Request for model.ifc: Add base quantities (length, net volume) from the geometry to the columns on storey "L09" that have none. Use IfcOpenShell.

First a look at what the model holds.

```python
import ifcopenshell
import ifcopenshell.util.element
import ifcopenshell.util.unit

model = ifcopenshell.open("model.ifc")
print(model.schema)
for unit_type in ("LENGTHUNIT", "AREAUNIT", "VOLUMEUNIT"):
    print(unit_type, ifcopenshell.util.unit.calculate_unit_scale(model, unit_type))
storey = next(s for s in model.by_type("IfcBuildingStorey") if s.Name == "L09")
columns = [e for e in ifcopenshell.util.element.get_decomposition(storey) if e.is_a("IfcColumn")]
for e in sorted(columns, key=lambda e: e.id()):
    print(e.id(), e.is_a(), e.Name, list(ifcopenshell.util.element.get_psets(e, qtos_only=True)), sep=" | ")
```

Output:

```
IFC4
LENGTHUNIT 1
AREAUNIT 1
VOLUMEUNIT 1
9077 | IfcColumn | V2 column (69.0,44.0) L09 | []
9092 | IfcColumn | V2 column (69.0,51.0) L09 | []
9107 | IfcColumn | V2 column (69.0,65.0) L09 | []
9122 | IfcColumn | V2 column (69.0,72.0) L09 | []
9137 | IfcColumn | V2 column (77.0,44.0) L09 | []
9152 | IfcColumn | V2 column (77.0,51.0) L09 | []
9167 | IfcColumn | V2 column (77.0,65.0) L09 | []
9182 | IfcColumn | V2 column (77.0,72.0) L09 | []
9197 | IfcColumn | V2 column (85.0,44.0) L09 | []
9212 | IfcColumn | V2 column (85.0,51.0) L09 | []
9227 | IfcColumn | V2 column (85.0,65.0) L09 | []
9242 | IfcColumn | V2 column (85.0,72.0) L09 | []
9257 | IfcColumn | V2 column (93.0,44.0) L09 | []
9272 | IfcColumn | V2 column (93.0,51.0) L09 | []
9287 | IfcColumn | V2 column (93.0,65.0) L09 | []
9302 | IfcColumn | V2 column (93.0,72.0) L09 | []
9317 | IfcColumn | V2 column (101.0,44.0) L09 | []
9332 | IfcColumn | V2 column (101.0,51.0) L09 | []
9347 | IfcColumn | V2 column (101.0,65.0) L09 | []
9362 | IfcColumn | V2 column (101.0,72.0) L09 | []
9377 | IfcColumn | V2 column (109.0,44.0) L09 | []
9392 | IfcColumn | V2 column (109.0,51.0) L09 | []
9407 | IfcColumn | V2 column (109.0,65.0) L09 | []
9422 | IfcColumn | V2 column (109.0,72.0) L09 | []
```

```python
import ifcopenshell
import ifcopenshell.api.pset
import ifcopenshell.geom
import ifcopenshell.util.element
import ifcopenshell.util.shape
import ifcopenshell.util.unit

model = ifcopenshell.open("model.ifc")
unit_scale = ifcopenshell.util.unit.calculate_unit_scale(model)
volume_scale = ifcopenshell.util.unit.calculate_unit_scale(model, "VOLUMEUNIT")
settings = ifcopenshell.geom.settings()

storey = next(s for s in model.by_type("IfcBuildingStorey") if s.Name == "L09")
columns = [e for e in ifcopenshell.util.element.get_decomposition(storey) if e.is_a("IfcColumn")]

for e in sorted(columns, key=lambda e: e.id()):
    if ifcopenshell.util.element.get_psets(e, qtos_only=True, should_inherit=False):
        continue
    # Geometry comes back in metres, in the element's own axes.
    shape = ifcopenshell.geom.create_shape(settings, e)
    values = {
        "Length": ifcopenshell.util.shape.get_z(shape.geometry) / unit_scale,
        "NetVolume": ifcopenshell.util.shape.get_volume(shape.geometry) / volume_scale,
    }
    qto = ifcopenshell.api.pset.add_qto(model, product=e, name="Qto_ColumnBaseQuantities")
    ifcopenshell.api.pset.edit_qto(model, qto=qto, properties=values)
    print(e.id(), {k: round(v, 3) for k, v in values.items()})

model.write("model_rev.ifc")
```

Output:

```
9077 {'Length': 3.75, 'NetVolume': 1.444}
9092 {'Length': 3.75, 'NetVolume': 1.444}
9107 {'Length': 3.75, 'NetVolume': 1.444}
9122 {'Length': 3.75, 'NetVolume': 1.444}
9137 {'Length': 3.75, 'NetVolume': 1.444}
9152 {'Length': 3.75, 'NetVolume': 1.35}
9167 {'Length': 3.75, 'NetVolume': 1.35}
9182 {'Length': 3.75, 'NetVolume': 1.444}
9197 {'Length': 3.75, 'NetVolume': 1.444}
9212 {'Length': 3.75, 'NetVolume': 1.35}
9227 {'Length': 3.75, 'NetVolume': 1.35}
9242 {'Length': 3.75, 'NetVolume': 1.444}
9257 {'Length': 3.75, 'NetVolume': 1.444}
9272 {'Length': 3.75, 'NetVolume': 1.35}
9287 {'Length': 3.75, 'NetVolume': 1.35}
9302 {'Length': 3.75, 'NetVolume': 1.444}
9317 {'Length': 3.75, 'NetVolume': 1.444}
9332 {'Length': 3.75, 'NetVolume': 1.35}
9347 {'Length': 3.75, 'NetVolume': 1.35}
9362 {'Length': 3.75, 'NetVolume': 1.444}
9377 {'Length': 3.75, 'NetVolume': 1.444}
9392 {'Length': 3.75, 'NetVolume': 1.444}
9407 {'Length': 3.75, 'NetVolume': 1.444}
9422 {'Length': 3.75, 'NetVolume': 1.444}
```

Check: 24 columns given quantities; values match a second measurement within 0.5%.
